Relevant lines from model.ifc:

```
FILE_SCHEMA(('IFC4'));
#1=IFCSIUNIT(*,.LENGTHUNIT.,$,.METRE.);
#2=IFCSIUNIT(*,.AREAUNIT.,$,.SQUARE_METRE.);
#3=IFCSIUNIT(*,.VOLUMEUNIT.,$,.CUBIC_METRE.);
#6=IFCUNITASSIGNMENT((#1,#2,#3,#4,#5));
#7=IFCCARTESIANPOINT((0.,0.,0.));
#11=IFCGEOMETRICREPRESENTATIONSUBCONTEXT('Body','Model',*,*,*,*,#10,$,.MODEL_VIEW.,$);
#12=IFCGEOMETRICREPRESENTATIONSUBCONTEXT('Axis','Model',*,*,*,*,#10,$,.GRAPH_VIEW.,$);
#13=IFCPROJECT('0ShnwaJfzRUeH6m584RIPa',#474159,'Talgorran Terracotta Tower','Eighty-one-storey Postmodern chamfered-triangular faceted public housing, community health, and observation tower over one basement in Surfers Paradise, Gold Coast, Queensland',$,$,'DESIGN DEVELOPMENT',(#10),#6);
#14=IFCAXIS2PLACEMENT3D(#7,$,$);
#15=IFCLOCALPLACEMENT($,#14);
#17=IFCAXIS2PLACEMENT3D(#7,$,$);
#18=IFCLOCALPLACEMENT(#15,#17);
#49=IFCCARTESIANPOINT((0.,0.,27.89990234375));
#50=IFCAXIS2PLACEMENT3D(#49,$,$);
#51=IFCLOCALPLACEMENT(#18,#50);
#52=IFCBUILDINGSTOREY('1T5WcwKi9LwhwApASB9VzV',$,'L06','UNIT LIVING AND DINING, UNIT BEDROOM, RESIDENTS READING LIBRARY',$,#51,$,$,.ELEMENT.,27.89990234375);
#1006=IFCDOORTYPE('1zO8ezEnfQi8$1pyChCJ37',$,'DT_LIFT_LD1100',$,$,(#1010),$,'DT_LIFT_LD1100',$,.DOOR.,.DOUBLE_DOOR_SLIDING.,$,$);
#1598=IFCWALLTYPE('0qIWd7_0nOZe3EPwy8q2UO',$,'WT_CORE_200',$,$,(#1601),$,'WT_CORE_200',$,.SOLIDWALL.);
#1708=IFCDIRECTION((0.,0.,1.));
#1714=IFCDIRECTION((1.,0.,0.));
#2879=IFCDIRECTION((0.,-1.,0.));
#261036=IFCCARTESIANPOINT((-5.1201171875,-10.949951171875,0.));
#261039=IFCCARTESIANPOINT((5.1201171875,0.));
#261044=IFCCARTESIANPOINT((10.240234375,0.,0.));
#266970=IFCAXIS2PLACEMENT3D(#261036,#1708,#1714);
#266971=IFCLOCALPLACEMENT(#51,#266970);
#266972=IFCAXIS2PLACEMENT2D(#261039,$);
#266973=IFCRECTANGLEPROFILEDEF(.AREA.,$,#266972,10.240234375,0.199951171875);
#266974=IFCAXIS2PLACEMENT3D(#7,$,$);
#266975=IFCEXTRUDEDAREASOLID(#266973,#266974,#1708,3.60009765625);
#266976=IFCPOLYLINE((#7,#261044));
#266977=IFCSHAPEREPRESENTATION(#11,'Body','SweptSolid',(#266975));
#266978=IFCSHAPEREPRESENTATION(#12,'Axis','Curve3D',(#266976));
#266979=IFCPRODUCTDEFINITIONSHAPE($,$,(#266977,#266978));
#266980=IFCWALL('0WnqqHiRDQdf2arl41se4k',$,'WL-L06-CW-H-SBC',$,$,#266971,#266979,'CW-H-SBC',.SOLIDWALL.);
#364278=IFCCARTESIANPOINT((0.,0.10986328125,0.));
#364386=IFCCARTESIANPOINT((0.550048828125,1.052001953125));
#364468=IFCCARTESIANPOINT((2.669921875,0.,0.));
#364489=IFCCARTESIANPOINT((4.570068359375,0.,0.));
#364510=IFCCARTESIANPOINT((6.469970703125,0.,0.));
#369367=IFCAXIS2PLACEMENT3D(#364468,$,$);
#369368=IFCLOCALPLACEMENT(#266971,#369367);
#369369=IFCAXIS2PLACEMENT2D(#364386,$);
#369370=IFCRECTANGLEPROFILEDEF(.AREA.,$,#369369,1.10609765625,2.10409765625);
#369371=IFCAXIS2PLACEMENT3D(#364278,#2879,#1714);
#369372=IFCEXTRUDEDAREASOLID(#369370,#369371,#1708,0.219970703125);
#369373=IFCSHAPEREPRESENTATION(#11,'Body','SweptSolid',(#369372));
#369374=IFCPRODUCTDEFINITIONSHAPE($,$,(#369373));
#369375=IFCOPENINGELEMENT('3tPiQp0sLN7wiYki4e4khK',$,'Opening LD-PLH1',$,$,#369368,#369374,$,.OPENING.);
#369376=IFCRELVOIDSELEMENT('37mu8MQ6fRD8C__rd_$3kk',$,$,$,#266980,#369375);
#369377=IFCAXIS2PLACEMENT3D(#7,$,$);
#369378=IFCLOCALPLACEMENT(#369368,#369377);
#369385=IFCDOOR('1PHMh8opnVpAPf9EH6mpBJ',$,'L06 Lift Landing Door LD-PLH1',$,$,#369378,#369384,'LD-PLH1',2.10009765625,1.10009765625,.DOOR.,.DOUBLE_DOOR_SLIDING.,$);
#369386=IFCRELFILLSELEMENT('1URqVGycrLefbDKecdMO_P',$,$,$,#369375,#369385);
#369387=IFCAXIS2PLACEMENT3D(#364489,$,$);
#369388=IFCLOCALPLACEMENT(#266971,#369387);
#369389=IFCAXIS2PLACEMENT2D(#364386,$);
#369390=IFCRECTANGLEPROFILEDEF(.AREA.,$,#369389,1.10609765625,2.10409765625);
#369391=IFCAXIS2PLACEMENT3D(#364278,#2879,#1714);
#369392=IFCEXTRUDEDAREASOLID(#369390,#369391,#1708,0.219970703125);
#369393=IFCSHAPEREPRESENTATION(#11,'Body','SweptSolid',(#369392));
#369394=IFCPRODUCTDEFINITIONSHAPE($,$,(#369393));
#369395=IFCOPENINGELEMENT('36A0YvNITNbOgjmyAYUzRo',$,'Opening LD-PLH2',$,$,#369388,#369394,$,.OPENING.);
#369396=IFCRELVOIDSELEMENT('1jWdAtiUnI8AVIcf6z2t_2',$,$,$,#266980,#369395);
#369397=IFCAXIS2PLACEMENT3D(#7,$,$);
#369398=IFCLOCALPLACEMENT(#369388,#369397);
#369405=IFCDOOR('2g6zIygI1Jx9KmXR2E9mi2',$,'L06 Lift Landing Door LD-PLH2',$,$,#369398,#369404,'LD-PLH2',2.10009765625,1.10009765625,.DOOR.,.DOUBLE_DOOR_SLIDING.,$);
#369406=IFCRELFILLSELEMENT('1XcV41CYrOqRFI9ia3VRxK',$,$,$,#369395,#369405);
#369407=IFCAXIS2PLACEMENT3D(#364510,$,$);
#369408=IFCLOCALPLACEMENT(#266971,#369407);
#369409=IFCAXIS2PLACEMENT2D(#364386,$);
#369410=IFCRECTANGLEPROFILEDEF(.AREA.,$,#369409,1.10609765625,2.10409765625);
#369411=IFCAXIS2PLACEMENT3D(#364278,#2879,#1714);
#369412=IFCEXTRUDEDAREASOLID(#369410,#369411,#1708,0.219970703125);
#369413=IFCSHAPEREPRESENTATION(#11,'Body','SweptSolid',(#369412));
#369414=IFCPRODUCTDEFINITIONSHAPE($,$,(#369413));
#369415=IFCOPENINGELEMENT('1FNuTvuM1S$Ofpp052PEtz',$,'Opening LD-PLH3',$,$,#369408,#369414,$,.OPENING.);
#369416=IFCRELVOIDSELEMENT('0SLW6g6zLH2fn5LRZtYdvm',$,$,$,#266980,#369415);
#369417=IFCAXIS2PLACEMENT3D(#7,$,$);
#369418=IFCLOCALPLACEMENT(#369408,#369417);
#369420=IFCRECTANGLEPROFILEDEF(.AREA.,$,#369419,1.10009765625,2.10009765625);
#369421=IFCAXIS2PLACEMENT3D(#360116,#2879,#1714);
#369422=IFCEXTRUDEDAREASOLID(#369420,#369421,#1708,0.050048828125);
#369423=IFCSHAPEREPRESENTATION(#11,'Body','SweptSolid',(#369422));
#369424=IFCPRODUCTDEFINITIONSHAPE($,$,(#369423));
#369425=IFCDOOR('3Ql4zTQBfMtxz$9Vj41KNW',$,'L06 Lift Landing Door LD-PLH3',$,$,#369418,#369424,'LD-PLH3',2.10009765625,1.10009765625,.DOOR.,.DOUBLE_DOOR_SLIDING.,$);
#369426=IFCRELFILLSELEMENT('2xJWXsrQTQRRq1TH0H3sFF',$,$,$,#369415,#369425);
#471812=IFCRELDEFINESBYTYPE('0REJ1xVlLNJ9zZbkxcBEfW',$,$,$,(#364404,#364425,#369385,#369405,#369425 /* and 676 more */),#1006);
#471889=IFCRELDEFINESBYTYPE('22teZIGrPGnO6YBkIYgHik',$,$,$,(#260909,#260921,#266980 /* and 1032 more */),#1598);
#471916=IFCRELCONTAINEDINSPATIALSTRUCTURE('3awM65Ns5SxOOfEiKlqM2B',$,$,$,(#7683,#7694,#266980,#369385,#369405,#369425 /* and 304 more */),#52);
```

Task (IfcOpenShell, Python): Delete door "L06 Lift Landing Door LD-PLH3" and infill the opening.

```python
import ifcopenshell
import ifcopenshell.api.feature
import ifcopenshell.api.root
import ifcopenshell.geom
import ifcopenshell.util.shape

model = ifcopenshell.open("model.ifc")
settings = ifcopenshell.geom.settings()


def volume(element):
    """Net volume in cubic metres, openings subtracted."""
    shape = ifcopenshell.geom.create_shape(settings, element)
    return ifcopenshell.util.shape.get_volume(shape.geometry)


door = model.by_guid("3Ql4zTQBfMtxz$9Vj41KNW")
opening = door.FillsVoids[0].RelatingOpeningElement
wall = opening.VoidsElements[0].RelatingBuildingElement
before = volume(wall)

ifcopenshell.api.root.remove_product(model, product=door)
ifcopenshell.api.feature.remove_feature(model, feature=opening)

after = volume(wall)

print(f"wall volume {before:.3f} -> {after:.3f} m3")

model.write("model_rev.ifc")
```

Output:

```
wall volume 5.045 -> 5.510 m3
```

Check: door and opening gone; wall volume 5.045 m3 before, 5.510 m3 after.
